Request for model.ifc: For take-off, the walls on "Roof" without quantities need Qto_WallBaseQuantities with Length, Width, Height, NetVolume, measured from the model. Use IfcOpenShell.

First a look at what the model holds.

```python
import ifcopenshell
import ifcopenshell.util.element
import ifcopenshell.util.unit

model = ifcopenshell.open("model.ifc")
print(model.schema)
for unit_type in ("LENGTHUNIT", "AREAUNIT", "VOLUMEUNIT"):
    print(unit_type, ifcopenshell.util.unit.calculate_unit_scale(model, unit_type))
storey = next(s for s in model.by_type("IfcBuildingStorey") if s.Name == "Roof")
walls = [e for e in ifcopenshell.util.element.get_decomposition(storey) if e.is_a("IfcWall")]
for e in sorted(walls, key=lambda e: e.id()):
    print(e.id(), e.is_a(), e.Name, list(ifcopenshell.util.element.get_psets(e, qtos_only=True)), sep=" | ")
```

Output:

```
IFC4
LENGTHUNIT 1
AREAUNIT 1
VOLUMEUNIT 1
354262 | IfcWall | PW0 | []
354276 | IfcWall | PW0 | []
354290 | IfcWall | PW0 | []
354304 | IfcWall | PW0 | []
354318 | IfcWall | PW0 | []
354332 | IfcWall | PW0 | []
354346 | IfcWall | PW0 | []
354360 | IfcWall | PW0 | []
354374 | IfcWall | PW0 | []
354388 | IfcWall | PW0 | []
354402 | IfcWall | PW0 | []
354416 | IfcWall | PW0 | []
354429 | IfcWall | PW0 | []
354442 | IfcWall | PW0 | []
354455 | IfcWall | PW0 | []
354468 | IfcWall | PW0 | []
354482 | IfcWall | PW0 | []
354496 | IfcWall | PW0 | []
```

```python
import ifcopenshell
import ifcopenshell.api.pset
import ifcopenshell.geom
import ifcopenshell.util.element
import ifcopenshell.util.shape
import ifcopenshell.util.unit

model = ifcopenshell.open("model.ifc")
unit_scale = ifcopenshell.util.unit.calculate_unit_scale(model)
volume_scale = ifcopenshell.util.unit.calculate_unit_scale(model, "VOLUMEUNIT")
settings = ifcopenshell.geom.settings()

storey = next(s for s in model.by_type("IfcBuildingStorey") if s.Name == "Roof")
walls = [e for e in ifcopenshell.util.element.get_decomposition(storey) if e.is_a("IfcWall")]

for e in sorted(walls, key=lambda e: e.id()):
    if ifcopenshell.util.element.get_psets(e, qtos_only=True, should_inherit=False):
        continue
    # Geometry comes back in metres, in the element's own axes.
    shape = ifcopenshell.geom.create_shape(settings, e)
    values = {
        "Length": ifcopenshell.util.shape.get_x(shape.geometry) / unit_scale,
        "Width": ifcopenshell.util.shape.get_y(shape.geometry) / unit_scale,
        "Height": ifcopenshell.util.shape.get_z(shape.geometry) / unit_scale,
        "NetVolume": ifcopenshell.util.shape.get_volume(shape.geometry) / volume_scale,
    }
    qto = ifcopenshell.api.pset.add_qto(model, product=e, name="Qto_WallBaseQuantities")
    ifcopenshell.api.pset.edit_qto(model, qto=qto, properties=values)
    print(e.id(), {k: round(v, 3) for k, v in values.items()})

model.write("model_edited.ifc")
```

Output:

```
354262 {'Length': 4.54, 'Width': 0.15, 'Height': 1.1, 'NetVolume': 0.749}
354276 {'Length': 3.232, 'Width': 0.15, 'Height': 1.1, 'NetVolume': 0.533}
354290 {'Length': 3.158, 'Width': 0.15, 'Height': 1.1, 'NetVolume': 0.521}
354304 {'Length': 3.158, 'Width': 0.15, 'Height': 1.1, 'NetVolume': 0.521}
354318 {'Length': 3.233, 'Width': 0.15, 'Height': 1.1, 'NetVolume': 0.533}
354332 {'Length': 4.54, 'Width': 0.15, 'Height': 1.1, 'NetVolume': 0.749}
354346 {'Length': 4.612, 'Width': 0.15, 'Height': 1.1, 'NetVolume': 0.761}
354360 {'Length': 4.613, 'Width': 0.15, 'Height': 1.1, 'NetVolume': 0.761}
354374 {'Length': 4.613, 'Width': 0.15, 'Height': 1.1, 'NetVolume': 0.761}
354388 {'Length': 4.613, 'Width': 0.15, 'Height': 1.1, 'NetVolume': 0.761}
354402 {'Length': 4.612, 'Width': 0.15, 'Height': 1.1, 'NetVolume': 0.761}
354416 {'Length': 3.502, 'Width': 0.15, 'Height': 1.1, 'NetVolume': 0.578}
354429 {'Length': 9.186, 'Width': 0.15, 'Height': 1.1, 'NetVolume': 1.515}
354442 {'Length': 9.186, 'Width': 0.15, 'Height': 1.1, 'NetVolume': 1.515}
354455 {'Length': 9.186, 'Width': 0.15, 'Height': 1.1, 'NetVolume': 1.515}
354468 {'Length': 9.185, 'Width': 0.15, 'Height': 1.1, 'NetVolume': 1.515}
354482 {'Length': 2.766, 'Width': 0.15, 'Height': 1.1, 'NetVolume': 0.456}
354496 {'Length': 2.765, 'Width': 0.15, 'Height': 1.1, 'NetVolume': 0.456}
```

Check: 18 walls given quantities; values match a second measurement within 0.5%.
